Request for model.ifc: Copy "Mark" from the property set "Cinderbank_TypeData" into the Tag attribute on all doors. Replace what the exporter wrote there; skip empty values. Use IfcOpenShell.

First a look at what the model holds.

```python
import ifcopenshell
import ifcopenshell.util.element

model = ifcopenshell.open("model.ifc")
print(model.schema)
doors = model.by_type("IfcDoor")
print(len(doors), "doors")
for e in doors[:8]:
    source = ifcopenshell.util.element.get_pset(e, "Cinderbank_TypeData", "Mark")
    target = e.Tag
    print(e.id(), repr(source), repr(target), sep=" | ")
```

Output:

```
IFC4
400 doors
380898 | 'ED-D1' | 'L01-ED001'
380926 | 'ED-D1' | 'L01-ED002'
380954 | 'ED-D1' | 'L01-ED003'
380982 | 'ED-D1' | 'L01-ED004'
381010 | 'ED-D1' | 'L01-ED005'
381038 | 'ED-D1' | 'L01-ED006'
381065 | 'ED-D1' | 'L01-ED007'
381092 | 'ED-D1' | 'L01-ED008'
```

```python
import ifcopenshell
import ifcopenshell.util.element

model = ifcopenshell.open("model.ifc")

count = 0
for e in model.by_type("IfcDoor"):
    value = ifcopenshell.util.element.get_pset(e, "Cinderbank_TypeData", "Mark")
    current = e.Tag
    if not value or not value.strip() or current == value:
        continue
    e.Tag = value
    count += 1

print(count, "doors updated")

model.write("model_updated.ifc")
```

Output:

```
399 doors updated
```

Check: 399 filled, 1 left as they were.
